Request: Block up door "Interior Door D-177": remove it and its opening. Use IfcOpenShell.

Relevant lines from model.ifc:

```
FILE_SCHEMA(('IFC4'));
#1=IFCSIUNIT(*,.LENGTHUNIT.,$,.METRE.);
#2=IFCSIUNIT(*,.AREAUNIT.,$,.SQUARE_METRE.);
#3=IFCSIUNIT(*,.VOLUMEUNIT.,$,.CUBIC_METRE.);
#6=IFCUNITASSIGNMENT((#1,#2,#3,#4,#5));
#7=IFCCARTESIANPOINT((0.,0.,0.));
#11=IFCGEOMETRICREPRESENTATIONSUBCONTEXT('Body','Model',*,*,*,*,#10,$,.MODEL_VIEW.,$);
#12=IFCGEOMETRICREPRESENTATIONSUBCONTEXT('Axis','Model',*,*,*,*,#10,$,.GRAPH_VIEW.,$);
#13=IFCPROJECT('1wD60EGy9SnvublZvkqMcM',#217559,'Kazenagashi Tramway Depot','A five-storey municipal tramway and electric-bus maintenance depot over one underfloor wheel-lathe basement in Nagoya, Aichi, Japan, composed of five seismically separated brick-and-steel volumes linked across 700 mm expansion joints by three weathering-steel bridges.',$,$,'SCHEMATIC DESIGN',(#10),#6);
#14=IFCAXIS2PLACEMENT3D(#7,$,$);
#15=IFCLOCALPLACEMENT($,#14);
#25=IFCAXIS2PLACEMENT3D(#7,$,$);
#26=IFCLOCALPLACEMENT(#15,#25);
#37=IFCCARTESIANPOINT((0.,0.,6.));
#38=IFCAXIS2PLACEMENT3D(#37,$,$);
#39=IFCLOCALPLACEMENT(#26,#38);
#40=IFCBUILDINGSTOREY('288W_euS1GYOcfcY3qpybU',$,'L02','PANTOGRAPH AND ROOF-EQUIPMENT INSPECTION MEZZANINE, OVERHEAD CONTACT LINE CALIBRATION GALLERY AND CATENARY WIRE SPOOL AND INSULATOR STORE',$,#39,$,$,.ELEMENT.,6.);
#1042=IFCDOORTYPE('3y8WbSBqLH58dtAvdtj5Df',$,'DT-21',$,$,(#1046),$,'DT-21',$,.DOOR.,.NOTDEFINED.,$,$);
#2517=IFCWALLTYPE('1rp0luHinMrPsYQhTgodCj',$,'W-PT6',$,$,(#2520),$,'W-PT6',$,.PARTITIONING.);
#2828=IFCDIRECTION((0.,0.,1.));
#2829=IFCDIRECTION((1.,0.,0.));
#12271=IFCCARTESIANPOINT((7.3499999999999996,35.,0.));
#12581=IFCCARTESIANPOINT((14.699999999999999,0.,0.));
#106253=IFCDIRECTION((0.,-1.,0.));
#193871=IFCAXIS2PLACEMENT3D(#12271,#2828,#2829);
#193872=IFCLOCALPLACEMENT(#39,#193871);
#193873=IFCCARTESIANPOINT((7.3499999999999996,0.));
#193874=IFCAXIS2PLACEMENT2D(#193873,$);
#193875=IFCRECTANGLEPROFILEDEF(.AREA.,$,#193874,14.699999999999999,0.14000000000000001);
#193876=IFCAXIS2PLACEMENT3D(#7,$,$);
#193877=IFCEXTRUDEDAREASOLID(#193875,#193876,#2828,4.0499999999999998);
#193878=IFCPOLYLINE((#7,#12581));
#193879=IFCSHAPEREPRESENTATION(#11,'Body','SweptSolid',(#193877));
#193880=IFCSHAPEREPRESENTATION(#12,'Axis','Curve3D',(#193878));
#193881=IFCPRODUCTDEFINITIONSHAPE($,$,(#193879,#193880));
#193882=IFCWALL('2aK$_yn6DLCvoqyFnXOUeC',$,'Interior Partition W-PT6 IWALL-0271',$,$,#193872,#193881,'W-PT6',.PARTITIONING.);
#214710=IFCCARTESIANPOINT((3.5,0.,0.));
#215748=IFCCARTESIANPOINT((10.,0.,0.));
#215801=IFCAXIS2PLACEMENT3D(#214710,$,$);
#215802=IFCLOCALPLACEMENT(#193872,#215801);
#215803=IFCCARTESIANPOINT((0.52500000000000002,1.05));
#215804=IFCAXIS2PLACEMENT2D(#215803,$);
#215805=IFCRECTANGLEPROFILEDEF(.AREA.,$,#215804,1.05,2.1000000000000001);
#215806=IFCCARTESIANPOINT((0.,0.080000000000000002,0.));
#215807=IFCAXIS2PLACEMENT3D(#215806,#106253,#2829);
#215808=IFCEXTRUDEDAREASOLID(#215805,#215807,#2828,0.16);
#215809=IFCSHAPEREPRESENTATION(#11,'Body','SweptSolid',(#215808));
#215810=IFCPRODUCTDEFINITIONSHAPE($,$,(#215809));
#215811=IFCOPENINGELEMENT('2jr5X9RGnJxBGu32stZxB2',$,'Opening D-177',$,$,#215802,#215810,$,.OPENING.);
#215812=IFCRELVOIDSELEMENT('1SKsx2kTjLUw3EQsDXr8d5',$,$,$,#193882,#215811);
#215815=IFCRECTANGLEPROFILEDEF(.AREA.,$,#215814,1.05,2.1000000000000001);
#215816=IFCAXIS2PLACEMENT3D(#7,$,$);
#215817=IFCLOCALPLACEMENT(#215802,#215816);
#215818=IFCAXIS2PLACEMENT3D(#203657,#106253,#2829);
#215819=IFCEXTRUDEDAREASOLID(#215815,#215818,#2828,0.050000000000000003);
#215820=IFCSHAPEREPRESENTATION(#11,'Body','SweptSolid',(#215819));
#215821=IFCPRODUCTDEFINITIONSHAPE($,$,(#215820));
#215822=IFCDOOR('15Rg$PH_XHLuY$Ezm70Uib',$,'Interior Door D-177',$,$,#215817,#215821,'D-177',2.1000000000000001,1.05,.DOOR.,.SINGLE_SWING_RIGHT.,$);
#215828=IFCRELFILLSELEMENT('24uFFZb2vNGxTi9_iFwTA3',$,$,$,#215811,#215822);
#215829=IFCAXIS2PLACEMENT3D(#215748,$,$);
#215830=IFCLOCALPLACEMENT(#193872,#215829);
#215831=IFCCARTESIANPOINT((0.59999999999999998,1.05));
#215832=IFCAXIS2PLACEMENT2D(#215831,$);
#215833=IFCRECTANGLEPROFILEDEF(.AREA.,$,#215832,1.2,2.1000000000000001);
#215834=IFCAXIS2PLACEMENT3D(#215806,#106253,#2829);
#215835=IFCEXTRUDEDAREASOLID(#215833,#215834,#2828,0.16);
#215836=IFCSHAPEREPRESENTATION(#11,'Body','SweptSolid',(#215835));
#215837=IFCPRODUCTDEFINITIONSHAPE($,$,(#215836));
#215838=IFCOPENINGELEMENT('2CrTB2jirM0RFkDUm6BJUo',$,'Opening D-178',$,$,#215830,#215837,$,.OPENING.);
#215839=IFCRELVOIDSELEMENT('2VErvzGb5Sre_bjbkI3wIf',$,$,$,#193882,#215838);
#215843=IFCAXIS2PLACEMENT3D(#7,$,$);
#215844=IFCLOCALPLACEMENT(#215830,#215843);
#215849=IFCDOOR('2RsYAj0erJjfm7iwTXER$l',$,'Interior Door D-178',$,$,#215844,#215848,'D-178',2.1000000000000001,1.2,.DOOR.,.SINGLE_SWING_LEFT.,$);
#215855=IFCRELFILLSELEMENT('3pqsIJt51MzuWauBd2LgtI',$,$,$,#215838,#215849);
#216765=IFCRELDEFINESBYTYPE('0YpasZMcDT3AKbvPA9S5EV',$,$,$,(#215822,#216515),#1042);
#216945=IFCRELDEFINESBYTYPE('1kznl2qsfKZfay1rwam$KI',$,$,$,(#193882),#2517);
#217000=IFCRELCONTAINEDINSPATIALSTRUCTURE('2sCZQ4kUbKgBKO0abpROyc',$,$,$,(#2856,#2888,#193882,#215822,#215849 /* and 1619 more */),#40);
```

```python
import ifcopenshell
import ifcopenshell.api.feature
import ifcopenshell.api.root
import ifcopenshell.geom
import ifcopenshell.util.shape

model = ifcopenshell.open("model.ifc")
settings = ifcopenshell.geom.settings()


def volume(element):
    """Net volume in cubic metres, openings subtracted."""
    shape = ifcopenshell.geom.create_shape(settings, element)
    return ifcopenshell.util.shape.get_volume(shape.geometry)


door = model.by_guid("15Rg$PH_XHLuY$Ezm70Uib")
opening = door.FillsVoids[0].RelatingOpeningElement
wall = opening.VoidsElements[0].RelatingBuildingElement
before = volume(wall)

ifcopenshell.api.root.remove_product(model, product=door)
ifcopenshell.api.feature.remove_feature(model, feature=opening)

after = volume(wall)

print(f"wall volume {before:.3f} -> {after:.3f} m3")

model.write("model_edited.ifc")
```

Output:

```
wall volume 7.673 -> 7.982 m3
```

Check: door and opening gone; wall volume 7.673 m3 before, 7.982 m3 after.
